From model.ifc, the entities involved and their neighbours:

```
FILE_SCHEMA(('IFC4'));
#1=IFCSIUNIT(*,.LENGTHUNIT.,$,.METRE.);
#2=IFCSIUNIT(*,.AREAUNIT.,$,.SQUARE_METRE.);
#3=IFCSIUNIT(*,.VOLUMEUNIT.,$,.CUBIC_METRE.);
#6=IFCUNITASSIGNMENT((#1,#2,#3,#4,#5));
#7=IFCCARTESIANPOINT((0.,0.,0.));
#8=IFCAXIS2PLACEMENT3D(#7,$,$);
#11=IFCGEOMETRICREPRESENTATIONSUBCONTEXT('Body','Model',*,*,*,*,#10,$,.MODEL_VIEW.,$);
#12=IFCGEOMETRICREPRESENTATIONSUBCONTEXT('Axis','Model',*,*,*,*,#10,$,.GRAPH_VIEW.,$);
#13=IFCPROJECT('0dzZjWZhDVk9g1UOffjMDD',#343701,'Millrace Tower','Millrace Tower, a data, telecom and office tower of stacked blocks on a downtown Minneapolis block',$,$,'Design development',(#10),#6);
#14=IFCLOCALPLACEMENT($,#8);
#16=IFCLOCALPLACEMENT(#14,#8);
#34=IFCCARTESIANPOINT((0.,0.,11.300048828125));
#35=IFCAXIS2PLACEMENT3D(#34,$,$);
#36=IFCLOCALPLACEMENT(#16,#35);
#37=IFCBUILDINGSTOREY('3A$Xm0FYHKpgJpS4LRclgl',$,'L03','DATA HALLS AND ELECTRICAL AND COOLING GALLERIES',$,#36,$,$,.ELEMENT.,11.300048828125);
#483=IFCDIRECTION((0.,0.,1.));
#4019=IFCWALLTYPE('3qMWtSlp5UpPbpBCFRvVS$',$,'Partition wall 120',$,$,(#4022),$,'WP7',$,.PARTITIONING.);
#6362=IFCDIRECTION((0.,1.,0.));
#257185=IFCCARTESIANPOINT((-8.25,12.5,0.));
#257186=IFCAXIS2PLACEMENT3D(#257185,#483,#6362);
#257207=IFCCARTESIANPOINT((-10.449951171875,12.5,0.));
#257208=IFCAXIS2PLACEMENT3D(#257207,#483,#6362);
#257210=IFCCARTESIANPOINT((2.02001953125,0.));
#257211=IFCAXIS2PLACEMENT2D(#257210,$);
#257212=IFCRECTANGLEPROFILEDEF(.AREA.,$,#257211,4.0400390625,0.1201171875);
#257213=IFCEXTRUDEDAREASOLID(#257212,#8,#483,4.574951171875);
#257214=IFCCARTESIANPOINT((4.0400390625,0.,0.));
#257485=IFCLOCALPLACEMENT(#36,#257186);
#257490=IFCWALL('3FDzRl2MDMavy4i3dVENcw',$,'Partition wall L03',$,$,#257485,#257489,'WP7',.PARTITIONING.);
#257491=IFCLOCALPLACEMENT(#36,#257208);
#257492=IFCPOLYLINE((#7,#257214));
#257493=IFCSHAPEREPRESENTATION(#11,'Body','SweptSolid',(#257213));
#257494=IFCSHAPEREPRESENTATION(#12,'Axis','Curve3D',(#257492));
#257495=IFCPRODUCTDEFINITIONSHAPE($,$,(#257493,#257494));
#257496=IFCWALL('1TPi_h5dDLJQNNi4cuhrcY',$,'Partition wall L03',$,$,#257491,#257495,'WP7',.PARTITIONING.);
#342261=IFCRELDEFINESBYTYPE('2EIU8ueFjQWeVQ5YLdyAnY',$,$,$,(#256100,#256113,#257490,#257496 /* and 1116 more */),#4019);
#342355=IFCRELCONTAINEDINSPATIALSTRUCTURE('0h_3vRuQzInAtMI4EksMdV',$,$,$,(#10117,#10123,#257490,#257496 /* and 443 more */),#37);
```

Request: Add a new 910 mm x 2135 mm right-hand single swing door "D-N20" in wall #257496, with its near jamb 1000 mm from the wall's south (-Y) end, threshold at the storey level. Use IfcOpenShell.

```python
import numpy as np
import ifcopenshell
import ifcopenshell.api.feature
import ifcopenshell.api.geometry
import ifcopenshell.api.root
import ifcopenshell.api.spatial
import ifcopenshell.geom
import ifcopenshell.util.element
import ifcopenshell.util.placement
import ifcopenshell.util.representation
import ifcopenshell.util.shape
import ifcopenshell.util.unit

model = ifcopenshell.open("model.ifc")
unit_scale = ifcopenshell.util.unit.calculate_unit_scale(model)
settings = ifcopenshell.geom.settings()


def volume(element):
    """Net volume in cubic metres, openings subtracted."""
    shape = ifcopenshell.geom.create_shape(settings, element)
    return ifcopenshell.util.shape.get_volume(shape.geometry)


wall = model.by_id(257496)
storey = ifcopenshell.util.element.get_container(wall, ifc_class="IfcBuildingStorey")
context = ifcopenshell.util.representation.get_context(model, "Model", "Body", "MODEL_VIEW")
before = volume(wall)

width, height, from_end, sill = 0.91, 2.135, 1, 0.0  # metres

# The wall runs along its own X axis, and the end named is its -X end.
wall_shape = ifcopenshell.geom.create_shape(settings, wall)
x, y, z = ifcopenshell.util.shape.get_vertices(wall_shape.geometry).T
start = x.min() + from_end
face, thickness = float(y.min()), float(y.max() - y.min())
wall_matrix = ifcopenshell.util.placement.get_local_placement(wall.ObjectPlacement)
level = ifcopenshell.util.placement.get_local_placement(storey.ObjectPlacement)[2, 3]


def in_wall(x, y):
    """Placement at x, y metres in the wall's axes, at sill height."""
    matrix = wall_matrix.copy()
    matrix[:, 3] = wall_matrix @ np.array([x / unit_scale, y / unit_scale, 0.0, 1.0])
    matrix[2, 3] = level + sill / unit_scale
    return matrix


# Opening: a box that overshoots both wall faces by 50 mm.
opening = ifcopenshell.api.root.create_entity(model, ifc_class="IfcOpeningElement", predefined_type="OPENING")
box = ifcopenshell.api.geometry.add_wall_representation(
    model, context=context, length=width, height=height, thickness=thickness + 0.1
)
ifcopenshell.api.geometry.assign_representation(model, product=opening, representation=box)
ifcopenshell.api.geometry.edit_object_placement(model, product=opening, matrix=in_wall(start, face - 0.05), is_si=False)
ifcopenshell.api.feature.add_feature(model, feature=opening, element=wall)

door = ifcopenshell.api.root.create_entity(model, ifc_class="IfcDoor", name="D-N20", predefined_type="DOOR")
door.OverallWidth, door.OverallHeight = width / unit_scale, height / unit_scale
door.OperationType = "SINGLE_SWING_RIGHT"
body = ifcopenshell.api.geometry.add_door_representation(
    model,
    context=context,
    overall_width=door.OverallWidth,
    overall_height=door.OverallHeight,
    operation_type="SINGLE_SWING_RIGHT",
    lining_properties={"LiningDepth": thickness / unit_scale, "ThresholdDepth": thickness / unit_scale},
)
ifcopenshell.api.geometry.assign_representation(model, product=door, representation=body)
ifcopenshell.api.spatial.assign_container(model, products=[door], relating_structure=storey)
ifcopenshell.api.feature.add_filling(model, opening=opening, element=door)

# The lining spans the wall, so the door starts at the wall face.
ifcopenshell.api.geometry.edit_object_placement(model, product=door, matrix=in_wall(start, face), is_si=False)

after = volume(wall)

print(f"wall volume {before:.3f} -> {after:.3f} m3")

model.write("model-out.ifc")
```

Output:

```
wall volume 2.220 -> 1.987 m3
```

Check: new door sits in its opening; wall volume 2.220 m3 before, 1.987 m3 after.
